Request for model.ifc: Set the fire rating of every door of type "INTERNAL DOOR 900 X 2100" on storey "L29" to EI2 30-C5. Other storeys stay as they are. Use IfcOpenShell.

First a look at what the model holds.

```python
import ifcopenshell
import ifcopenshell.util.element

model = ifcopenshell.open("model.ifc")
print(model.schema)
storey = next(s for s in model.by_type("IfcBuildingStorey") if s.Name == "L29")
doors = [e for e in ifcopenshell.util.element.get_decomposition(storey) if e.is_a("IfcDoor")]
seen = {}
for e in doors:
    element_type = ifcopenshell.util.element.get_type(e)
    key = (element_type.Name if element_type != e and element_type else None, ifcopenshell.util.element.get_pset(e, "Pset_DoorCommon", "FireRating"))
    seen[key] = seen.get(key, 0) + 1
for (name, value), count in sorted(seen.items(), key=str):
    print(count, "x", name, "|", value)
```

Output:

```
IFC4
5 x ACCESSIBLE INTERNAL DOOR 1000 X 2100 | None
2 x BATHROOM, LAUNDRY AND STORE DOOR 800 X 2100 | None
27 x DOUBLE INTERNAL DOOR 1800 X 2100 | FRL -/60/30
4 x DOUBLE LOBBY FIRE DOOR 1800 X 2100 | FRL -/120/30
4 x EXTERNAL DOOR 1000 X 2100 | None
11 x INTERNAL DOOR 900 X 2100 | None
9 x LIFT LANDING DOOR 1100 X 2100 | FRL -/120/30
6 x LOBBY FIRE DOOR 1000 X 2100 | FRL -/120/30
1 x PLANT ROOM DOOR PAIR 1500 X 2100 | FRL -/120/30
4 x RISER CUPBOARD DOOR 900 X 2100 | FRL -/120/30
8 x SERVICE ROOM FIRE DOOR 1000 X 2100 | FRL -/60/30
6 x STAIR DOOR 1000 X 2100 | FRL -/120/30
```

```python
import ifcopenshell
import ifcopenshell.api.pset
import ifcopenshell.util.element

model = ifcopenshell.open("model.ifc")

storey = next(s for s in model.by_type("IfcBuildingStorey") if s.Name == "L29")
doors = [e for e in ifcopenshell.util.element.get_decomposition(storey) if e.is_a("IfcDoor")]

count = 0
for e in doors:
    element_type = ifcopenshell.util.element.get_type(e)
    if element_type in (None, e) or element_type.Name != "INTERNAL DOOR 900 X 2100":
        continue
    found = ifcopenshell.util.element.get_pset(e, "Pset_DoorCommon", should_inherit=False)
    if found:
        pset = model.by_id(found["id"])
        if len(ifcopenshell.util.element.get_elements_by_pset(pset)) > 1:
            pset = ifcopenshell.api.pset.unshare_pset(model, products=[e], pset=pset)[0]
    else:
        pset = ifcopenshell.api.pset.add_pset(model, product=e, name="Pset_DoorCommon")
    ifcopenshell.api.pset.edit_pset(model, pset=pset, properties={"FireRating": "EI2 30-C5"})
    count += 1

print(count, "doors updated")

model.write("model_updated.ifc")
```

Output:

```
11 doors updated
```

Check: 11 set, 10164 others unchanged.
